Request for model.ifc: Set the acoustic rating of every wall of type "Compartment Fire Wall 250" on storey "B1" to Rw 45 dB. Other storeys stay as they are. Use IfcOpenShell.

First a look at what the model holds.

```python
import ifcopenshell
import ifcopenshell.util.element

model = ifcopenshell.open("model.ifc")
print(model.schema)
storey = next(s for s in model.by_type("IfcBuildingStorey") if s.Name == "B1")
walls = [e for e in ifcopenshell.util.element.get_decomposition(storey) if e.is_a("IfcWall")]
seen = {}
for e in walls:
    element_type = ifcopenshell.util.element.get_type(e)
    key = (element_type.Name if element_type != e and element_type else None, ifcopenshell.util.element.get_pset(e, "Pset_WallCommon", "AcousticRating"))
    seen[key] = seen.get(key, 0) + 1
for (name, value), count in sorted(seen.items(), key=str):
    print(count, "x", name, "|", value)
```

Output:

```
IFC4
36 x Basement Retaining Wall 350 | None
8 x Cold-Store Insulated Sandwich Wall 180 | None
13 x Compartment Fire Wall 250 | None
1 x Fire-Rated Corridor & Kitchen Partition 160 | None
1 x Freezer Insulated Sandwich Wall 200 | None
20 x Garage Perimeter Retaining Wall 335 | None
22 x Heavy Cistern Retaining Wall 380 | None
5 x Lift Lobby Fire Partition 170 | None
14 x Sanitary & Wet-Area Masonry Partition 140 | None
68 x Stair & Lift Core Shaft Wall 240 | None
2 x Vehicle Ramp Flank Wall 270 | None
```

```python
import ifcopenshell
import ifcopenshell.api.pset
import ifcopenshell.util.element

model = ifcopenshell.open("model.ifc")

storey = next(s for s in model.by_type("IfcBuildingStorey") if s.Name == "B1")
walls = [e for e in ifcopenshell.util.element.get_decomposition(storey) if e.is_a("IfcWall")]

count = 0
for e in walls:
    element_type = ifcopenshell.util.element.get_type(e)
    if element_type in (None, e) or element_type.Name != "Compartment Fire Wall 250":
        continue
    # add_pset returns the element's existing set when there is one.
    pset = ifcopenshell.api.pset.add_pset(model, product=e, name="Pset_WallCommon")
    ifcopenshell.api.pset.edit_pset(model, pset=pset, properties={"AcousticRating": "Rw 45 dB"})
    count += 1

print(count, "walls updated")

model.write("model-out.ifc")
```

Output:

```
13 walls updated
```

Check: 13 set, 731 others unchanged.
